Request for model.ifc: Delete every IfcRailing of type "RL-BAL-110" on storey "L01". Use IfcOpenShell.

First a look at what the model holds.

```python
import ifcopenshell
import ifcopenshell.util.element

model = ifcopenshell.open("model.ifc")
print(model.schema)
storey = next(s for s in model.by_type("IfcBuildingStorey") if s.Name == "L01")
railings = [e for e in ifcopenshell.util.element.get_decomposition(storey) if e.is_a("IfcRailing")]
seen = {}
for e in railings:
    element_type = ifcopenshell.util.element.get_type(e)
    name = element_type.Name if element_type not in (None, e) else None
    seen[name] = seen.get(name, 0) + 1
for name, count in sorted(seen.items(), key=str):
    print(count, "x", name)
```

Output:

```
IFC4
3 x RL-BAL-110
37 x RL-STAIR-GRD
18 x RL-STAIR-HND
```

```python
import ifcopenshell
import ifcopenshell.api.root
import ifcopenshell.util.element

model = ifcopenshell.open("model.ifc")

storey = next(s for s in model.by_type("IfcBuildingStorey") if s.Name == "L01")
railings = [e for e in ifcopenshell.util.element.get_decomposition(storey) if e.is_a("IfcRailing")]
targets = [e for e in railings if (t := ifcopenshell.util.element.get_type(e)) not in (None, e) and t.Name == "RL-BAL-110"]

for e in targets:
    ifcopenshell.api.root.remove_product(model, product=e)
print(len(targets), "removed")

model.write("model_rev.ifc")
```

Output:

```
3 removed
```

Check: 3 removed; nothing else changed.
